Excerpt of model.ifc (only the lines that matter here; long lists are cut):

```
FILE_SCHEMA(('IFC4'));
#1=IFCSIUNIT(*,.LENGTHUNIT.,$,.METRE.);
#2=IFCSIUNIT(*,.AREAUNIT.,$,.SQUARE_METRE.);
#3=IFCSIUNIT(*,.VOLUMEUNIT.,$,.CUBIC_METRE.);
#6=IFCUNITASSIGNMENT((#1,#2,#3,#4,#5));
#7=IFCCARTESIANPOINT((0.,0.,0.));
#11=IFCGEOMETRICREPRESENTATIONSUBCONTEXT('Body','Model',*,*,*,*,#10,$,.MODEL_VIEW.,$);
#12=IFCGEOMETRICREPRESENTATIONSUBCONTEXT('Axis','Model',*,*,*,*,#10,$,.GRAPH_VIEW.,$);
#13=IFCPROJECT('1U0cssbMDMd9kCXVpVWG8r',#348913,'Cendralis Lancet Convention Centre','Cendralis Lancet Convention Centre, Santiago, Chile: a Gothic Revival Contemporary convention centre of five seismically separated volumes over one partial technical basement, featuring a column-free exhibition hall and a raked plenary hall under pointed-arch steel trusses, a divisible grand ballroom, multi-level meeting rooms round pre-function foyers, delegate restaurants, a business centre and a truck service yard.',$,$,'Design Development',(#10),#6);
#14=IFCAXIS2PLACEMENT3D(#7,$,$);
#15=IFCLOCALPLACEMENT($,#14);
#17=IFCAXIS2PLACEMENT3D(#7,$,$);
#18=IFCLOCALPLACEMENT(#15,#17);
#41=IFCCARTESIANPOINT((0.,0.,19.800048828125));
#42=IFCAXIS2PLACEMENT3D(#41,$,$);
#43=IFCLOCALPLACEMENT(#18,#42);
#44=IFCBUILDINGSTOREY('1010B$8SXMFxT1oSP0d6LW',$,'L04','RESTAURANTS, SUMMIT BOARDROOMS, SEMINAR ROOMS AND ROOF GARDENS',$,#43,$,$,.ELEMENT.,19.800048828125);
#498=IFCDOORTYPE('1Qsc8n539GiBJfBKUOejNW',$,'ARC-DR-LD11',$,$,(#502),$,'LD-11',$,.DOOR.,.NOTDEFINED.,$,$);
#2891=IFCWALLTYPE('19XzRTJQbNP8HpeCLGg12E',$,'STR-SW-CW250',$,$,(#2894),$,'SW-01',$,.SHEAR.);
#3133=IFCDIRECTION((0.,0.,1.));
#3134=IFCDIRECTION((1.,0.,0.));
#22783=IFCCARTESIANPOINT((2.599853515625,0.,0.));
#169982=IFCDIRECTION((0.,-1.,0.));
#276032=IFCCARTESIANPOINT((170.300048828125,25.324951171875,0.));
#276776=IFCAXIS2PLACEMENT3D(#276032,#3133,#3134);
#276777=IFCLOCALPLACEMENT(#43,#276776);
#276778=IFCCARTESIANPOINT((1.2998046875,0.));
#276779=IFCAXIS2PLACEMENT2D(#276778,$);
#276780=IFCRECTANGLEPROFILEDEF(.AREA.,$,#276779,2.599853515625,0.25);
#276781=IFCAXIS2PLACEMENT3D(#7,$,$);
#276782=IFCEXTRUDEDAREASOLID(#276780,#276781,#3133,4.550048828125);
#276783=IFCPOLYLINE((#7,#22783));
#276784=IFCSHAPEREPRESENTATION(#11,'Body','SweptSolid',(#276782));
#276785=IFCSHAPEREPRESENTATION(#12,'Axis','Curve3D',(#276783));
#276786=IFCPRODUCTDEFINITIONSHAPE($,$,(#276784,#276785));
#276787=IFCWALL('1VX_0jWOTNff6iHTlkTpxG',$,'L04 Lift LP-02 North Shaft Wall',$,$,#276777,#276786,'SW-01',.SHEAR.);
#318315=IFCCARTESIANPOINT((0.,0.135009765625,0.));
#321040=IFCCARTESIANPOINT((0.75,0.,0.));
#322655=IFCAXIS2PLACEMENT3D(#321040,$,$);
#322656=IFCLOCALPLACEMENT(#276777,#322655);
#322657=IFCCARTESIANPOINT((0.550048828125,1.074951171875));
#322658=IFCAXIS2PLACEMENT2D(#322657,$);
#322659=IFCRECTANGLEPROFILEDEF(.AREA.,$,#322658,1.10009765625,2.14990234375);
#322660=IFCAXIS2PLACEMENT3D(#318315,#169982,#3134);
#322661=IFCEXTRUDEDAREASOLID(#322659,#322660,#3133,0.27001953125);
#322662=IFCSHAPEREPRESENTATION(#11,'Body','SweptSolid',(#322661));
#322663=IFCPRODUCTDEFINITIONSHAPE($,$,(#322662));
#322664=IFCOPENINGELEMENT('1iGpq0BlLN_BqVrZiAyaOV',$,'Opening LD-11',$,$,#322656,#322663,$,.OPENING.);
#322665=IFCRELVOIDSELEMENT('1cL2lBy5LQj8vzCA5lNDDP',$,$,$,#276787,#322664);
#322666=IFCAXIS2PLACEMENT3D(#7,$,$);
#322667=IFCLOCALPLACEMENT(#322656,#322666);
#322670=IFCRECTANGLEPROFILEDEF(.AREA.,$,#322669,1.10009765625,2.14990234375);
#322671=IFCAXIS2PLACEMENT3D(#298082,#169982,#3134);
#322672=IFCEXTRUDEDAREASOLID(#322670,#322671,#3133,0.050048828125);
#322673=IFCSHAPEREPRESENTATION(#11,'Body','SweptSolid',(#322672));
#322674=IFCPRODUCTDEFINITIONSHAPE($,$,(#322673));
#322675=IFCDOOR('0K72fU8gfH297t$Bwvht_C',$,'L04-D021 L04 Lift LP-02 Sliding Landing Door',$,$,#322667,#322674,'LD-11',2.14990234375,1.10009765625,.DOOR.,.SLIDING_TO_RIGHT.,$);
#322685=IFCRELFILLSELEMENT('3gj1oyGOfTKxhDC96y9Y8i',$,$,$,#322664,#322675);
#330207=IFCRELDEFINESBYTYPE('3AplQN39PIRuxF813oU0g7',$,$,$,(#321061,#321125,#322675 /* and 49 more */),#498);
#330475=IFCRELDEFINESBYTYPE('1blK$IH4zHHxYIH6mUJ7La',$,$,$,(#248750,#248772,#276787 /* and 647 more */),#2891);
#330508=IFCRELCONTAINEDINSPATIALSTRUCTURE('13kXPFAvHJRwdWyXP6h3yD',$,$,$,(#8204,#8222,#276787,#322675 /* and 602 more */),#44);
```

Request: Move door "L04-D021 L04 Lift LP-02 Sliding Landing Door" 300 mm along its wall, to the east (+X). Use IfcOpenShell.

```python
import ifcopenshell
import ifcopenshell.api.geometry
import ifcopenshell.util.placement

model = ifcopenshell.open("model.ifc")

door = model.by_guid("0K72fU8gfH297t$Bwvht_C")
opening = door.FillsVoids[0].RelatingOpeningElement
wall = opening.VoidsElements[0].RelatingBuildingElement

wall_matrix = ifcopenshell.util.placement.get_local_placement(wall.ObjectPlacement)
shift = wall_matrix[:3, 0] * 0.3
before = ifcopenshell.util.placement.get_local_placement(door.ObjectPlacement)[:3, 3].copy()

# The door is placed relative to its opening, so it follows when the opening moves.
matrix = ifcopenshell.util.placement.get_local_placement(opening.ObjectPlacement)
matrix[:3, 3] += shift
ifcopenshell.api.geometry.edit_object_placement(
    model, product=opening, matrix=matrix, is_si=False, should_transform_children=True
)

after = ifcopenshell.util.placement.get_local_placement(door.ObjectPlacement)[:3, 3]
print("door moved by", (after - before).round(3) + 0.0)

model.write("model_rev.ifc")
```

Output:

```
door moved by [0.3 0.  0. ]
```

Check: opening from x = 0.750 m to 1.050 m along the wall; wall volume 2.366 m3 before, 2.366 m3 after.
